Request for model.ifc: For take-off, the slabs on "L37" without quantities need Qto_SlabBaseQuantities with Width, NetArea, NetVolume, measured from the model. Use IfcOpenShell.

First a look at what the model holds.

```python
import ifcopenshell
import ifcopenshell.util.element
import ifcopenshell.util.unit

model = ifcopenshell.open("model.ifc")
print(model.schema)
for unit_type in ("LENGTHUNIT", "AREAUNIT", "VOLUMEUNIT"):
    print(unit_type, ifcopenshell.util.unit.calculate_unit_scale(model, unit_type))
storey = next(s for s in model.by_type("IfcBuildingStorey") if s.Name == "L37")
slabs = [e for e in ifcopenshell.util.element.get_decomposition(storey) if e.is_a("IfcSlab")]
for e in sorted(slabs, key=lambda e: e.id()):
    print(e.id(), e.is_a(), e.Name, list(ifcopenshell.util.element.get_psets(e, qtos_only=True)), sep=" | ")
```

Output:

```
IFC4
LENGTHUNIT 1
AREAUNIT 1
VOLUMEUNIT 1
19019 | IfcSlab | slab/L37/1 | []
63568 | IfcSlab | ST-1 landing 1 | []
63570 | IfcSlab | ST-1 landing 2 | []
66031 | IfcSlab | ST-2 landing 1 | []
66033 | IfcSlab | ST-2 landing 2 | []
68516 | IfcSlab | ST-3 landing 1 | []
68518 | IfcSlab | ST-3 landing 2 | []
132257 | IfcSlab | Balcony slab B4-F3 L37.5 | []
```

```python
import ifcopenshell
import ifcopenshell.api.pset
import ifcopenshell.geom
import ifcopenshell.util.element
import ifcopenshell.util.shape
import ifcopenshell.util.unit

model = ifcopenshell.open("model.ifc")
unit_scale = ifcopenshell.util.unit.calculate_unit_scale(model)
area_scale = ifcopenshell.util.unit.calculate_unit_scale(model, "AREAUNIT")
volume_scale = ifcopenshell.util.unit.calculate_unit_scale(model, "VOLUMEUNIT")
settings = ifcopenshell.geom.settings()

storey = next(s for s in model.by_type("IfcBuildingStorey") if s.Name == "L37")
slabs = [e for e in ifcopenshell.util.element.get_decomposition(storey) if e.is_a("IfcSlab")]

for e in sorted(slabs, key=lambda e: e.id()):
    if ifcopenshell.util.element.get_psets(e, qtos_only=True, should_inherit=False):
        continue
    # Geometry comes back in metres, in the element's own axes.
    shape = ifcopenshell.geom.create_shape(settings, e)
    values = {
        "Width": ifcopenshell.util.shape.get_z(shape.geometry) / unit_scale,
        "NetArea": ifcopenshell.util.shape.get_footprint_area(shape.geometry) / area_scale,
        "NetVolume": ifcopenshell.util.shape.get_volume(shape.geometry) / volume_scale,
    }
    qto = ifcopenshell.api.pset.add_qto(model, product=e, name="Qto_SlabBaseQuantities")
    ifcopenshell.api.pset.edit_qto(model, qto=qto, properties=values)
    print(e.id(), {k: round(v, 3) for k, v in values.items()})

model.write("model_v2.ifc")
```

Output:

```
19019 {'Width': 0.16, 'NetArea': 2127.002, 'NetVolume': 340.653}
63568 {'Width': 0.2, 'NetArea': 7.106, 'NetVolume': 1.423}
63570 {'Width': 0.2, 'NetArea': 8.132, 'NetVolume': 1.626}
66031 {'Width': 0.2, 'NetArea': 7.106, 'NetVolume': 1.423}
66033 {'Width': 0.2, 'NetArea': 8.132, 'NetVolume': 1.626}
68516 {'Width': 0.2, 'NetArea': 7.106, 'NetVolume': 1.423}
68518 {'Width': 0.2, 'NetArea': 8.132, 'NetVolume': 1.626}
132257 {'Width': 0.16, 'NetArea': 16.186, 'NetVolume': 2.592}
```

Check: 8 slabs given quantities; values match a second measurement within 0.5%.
